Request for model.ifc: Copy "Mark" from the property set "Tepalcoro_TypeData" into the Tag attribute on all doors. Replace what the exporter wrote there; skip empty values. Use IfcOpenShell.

First a look at what the model holds.

```python
import ifcopenshell
import ifcopenshell.util.element

model = ifcopenshell.open("model.ifc")
print(model.schema)
doors = model.by_type("IfcDoor")
print(len(doors), "doors")
for e in doors[:8]:
    source = ifcopenshell.util.element.get_pset(e, "Tepalcoro_TypeData", "Mark")
    target = e.Tag
    print(e.id(), repr(source), repr(target), sep=" | ")
```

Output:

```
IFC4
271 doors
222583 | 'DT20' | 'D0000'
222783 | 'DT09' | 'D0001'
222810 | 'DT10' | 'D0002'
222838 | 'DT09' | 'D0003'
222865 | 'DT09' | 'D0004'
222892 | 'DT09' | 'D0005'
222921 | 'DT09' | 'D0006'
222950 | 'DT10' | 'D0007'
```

```python
import ifcopenshell
import ifcopenshell.util.element

model = ifcopenshell.open("model.ifc")

count = 0
for e in model.by_type("IfcDoor"):
    value = ifcopenshell.util.element.get_pset(e, "Tepalcoro_TypeData", "Mark")
    current = e.Tag
    if not value or not value.strip() or current == value:
        continue
    e.Tag = value
    count += 1

print(count, "doors updated")

model.write("model-out.ifc")
```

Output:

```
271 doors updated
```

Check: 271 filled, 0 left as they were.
